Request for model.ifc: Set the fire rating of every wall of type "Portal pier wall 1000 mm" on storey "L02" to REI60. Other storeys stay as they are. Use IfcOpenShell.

First a look at what the model holds.

```python
import ifcopenshell
import ifcopenshell.util.element

model = ifcopenshell.open("model.ifc")
print(model.schema)
storey = next(s for s in model.by_type("IfcBuildingStorey") if s.Name == "L02")
walls = [e for e in ifcopenshell.util.element.get_decomposition(storey) if e.is_a("IfcWall")]
seen = {}
for e in walls:
    element_type = ifcopenshell.util.element.get_type(e)
    key = (element_type.Name if element_type != e and element_type else None, ifcopenshell.util.element.get_pset(e, "Pset_WallCommon", "FireRating"))
    seen[key] = seen.get(key, 0) + 1
for (name, value), count in sorted(seen.items(), key=str):
    print(count, "x", name, "|", value)
```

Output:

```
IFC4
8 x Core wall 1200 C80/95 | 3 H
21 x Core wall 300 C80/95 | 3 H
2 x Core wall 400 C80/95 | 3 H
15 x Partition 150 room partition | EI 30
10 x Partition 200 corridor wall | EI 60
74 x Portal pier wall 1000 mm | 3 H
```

```python
import ifcopenshell
import ifcopenshell.api.pset
import ifcopenshell.util.element

model = ifcopenshell.open("model.ifc")

storey = next(s for s in model.by_type("IfcBuildingStorey") if s.Name == "L02")
walls = [e for e in ifcopenshell.util.element.get_decomposition(storey) if e.is_a("IfcWall")]

count = 0
for e in walls:
    element_type = ifcopenshell.util.element.get_type(e)
    if element_type in (None, e) or element_type.Name != "Portal pier wall 1000 mm":
        continue
    found = ifcopenshell.util.element.get_pset(e, "Pset_WallCommon", should_inherit=False)
    if found:
        pset = model.by_id(found["id"])
        if len(ifcopenshell.util.element.get_elements_by_pset(pset)) > 1:
            pset = ifcopenshell.api.pset.unshare_pset(model, products=[e], pset=pset)[0]
    else:
        pset = ifcopenshell.api.pset.add_pset(model, product=e, name="Pset_WallCommon")
    ifcopenshell.api.pset.edit_pset(model, pset=pset, properties={"FireRating": "REI60"})
    count += 1

print(count, "walls updated")

model.write("model-out.ifc")
```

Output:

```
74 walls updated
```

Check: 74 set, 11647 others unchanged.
